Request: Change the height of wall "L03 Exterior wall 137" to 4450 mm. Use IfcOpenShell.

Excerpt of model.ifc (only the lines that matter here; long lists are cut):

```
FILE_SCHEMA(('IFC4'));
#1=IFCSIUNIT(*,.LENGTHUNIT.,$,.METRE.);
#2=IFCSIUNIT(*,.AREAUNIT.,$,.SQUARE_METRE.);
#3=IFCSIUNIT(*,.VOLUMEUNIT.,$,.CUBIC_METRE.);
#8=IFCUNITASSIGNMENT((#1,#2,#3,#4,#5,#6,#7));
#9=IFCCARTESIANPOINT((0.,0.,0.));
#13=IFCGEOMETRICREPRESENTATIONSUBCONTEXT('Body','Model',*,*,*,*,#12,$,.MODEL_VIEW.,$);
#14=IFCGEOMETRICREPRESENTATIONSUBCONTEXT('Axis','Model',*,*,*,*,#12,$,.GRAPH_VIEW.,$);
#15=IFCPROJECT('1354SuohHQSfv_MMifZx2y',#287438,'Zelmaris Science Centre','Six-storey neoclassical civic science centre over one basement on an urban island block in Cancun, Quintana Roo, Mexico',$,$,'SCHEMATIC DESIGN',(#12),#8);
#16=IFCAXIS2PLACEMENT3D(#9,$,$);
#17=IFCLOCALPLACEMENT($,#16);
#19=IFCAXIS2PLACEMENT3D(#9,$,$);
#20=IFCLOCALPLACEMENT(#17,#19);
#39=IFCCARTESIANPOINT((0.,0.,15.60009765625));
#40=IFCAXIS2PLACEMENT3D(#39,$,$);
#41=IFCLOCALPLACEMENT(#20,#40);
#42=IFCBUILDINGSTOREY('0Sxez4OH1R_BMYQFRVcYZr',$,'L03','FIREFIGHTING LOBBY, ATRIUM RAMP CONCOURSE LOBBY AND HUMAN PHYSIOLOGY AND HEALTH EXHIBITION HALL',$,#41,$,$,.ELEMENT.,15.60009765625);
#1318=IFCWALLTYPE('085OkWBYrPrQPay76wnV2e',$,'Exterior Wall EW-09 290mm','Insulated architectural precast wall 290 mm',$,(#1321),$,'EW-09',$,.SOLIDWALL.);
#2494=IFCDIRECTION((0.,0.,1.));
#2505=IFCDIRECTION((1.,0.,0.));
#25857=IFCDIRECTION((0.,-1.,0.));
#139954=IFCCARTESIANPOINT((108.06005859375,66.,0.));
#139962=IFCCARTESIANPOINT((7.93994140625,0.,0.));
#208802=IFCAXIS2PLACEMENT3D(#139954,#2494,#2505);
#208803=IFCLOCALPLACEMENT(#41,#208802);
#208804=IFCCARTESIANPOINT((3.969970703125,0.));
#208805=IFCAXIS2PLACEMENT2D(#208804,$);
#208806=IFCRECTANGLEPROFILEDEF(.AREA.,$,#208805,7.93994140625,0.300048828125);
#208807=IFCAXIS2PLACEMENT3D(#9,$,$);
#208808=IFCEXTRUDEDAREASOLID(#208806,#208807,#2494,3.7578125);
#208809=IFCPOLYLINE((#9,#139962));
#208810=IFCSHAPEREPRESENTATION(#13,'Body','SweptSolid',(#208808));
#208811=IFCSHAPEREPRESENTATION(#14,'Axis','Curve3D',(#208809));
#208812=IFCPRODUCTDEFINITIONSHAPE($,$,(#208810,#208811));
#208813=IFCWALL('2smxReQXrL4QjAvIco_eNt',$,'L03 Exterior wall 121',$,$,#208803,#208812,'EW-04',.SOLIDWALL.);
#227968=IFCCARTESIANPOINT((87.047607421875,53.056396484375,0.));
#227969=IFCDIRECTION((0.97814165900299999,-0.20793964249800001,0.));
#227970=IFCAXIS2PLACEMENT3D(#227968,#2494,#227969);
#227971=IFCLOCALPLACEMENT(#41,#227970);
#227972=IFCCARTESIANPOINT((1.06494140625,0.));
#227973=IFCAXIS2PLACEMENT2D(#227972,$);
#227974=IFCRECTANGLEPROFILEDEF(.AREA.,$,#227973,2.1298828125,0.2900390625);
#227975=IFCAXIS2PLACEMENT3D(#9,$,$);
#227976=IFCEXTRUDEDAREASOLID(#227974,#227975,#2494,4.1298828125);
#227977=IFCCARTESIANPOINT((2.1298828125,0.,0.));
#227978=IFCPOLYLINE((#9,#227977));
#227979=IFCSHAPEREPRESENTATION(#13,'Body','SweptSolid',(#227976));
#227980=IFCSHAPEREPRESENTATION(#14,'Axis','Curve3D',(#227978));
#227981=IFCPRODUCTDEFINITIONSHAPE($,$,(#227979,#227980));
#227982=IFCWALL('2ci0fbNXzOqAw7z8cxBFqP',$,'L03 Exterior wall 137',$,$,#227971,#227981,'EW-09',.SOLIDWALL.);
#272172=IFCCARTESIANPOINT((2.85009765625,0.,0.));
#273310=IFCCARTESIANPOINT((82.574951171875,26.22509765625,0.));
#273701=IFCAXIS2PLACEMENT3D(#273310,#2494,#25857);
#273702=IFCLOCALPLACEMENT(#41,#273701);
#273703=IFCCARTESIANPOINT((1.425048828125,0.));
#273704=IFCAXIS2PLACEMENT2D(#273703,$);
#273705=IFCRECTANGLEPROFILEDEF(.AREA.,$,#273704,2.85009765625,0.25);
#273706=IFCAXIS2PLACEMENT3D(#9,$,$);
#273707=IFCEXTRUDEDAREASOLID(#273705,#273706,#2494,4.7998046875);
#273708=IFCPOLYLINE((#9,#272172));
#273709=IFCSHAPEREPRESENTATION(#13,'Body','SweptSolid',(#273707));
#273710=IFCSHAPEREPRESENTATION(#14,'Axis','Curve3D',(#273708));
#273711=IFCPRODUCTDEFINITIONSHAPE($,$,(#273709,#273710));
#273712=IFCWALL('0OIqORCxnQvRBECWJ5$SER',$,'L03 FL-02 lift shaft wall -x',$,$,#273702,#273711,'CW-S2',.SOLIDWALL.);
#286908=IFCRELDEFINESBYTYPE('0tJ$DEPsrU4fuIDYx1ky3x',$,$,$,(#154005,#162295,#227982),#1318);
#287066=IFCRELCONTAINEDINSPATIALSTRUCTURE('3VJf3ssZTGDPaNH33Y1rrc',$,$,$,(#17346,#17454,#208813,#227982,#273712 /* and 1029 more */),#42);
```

```python
import ifcopenshell
import ifcopenshell.geom
import ifcopenshell.util.representation
import ifcopenshell.util.shape
import ifcopenshell.util.unit

model = ifcopenshell.open("model.ifc")
unit_scale = ifcopenshell.util.unit.calculate_unit_scale(model)
settings = ifcopenshell.geom.settings()


def volume(element):
    """Net volume in cubic metres, openings subtracted."""
    shape = ifcopenshell.geom.create_shape(settings, element)
    return ifcopenshell.util.shape.get_volume(shape.geometry)


wall = model.by_guid("2ci0fbNXzOqAw7z8cxBFqP")
before = volume(wall)

body = ifcopenshell.util.representation.get_representation(wall, "Model", "Body")
solid = body.Items[0]
old_height = solid.Depth
solid.Depth = 4.45 / unit_scale
after = volume(wall)

print(f"height {old_height:g} -> {solid.Depth:g}, volume {before:.3f} -> {after:.3f} m3")

model.write("model_rev.ifc")
```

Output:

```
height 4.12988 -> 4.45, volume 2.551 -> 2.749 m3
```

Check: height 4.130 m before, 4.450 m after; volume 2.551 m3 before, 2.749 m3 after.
